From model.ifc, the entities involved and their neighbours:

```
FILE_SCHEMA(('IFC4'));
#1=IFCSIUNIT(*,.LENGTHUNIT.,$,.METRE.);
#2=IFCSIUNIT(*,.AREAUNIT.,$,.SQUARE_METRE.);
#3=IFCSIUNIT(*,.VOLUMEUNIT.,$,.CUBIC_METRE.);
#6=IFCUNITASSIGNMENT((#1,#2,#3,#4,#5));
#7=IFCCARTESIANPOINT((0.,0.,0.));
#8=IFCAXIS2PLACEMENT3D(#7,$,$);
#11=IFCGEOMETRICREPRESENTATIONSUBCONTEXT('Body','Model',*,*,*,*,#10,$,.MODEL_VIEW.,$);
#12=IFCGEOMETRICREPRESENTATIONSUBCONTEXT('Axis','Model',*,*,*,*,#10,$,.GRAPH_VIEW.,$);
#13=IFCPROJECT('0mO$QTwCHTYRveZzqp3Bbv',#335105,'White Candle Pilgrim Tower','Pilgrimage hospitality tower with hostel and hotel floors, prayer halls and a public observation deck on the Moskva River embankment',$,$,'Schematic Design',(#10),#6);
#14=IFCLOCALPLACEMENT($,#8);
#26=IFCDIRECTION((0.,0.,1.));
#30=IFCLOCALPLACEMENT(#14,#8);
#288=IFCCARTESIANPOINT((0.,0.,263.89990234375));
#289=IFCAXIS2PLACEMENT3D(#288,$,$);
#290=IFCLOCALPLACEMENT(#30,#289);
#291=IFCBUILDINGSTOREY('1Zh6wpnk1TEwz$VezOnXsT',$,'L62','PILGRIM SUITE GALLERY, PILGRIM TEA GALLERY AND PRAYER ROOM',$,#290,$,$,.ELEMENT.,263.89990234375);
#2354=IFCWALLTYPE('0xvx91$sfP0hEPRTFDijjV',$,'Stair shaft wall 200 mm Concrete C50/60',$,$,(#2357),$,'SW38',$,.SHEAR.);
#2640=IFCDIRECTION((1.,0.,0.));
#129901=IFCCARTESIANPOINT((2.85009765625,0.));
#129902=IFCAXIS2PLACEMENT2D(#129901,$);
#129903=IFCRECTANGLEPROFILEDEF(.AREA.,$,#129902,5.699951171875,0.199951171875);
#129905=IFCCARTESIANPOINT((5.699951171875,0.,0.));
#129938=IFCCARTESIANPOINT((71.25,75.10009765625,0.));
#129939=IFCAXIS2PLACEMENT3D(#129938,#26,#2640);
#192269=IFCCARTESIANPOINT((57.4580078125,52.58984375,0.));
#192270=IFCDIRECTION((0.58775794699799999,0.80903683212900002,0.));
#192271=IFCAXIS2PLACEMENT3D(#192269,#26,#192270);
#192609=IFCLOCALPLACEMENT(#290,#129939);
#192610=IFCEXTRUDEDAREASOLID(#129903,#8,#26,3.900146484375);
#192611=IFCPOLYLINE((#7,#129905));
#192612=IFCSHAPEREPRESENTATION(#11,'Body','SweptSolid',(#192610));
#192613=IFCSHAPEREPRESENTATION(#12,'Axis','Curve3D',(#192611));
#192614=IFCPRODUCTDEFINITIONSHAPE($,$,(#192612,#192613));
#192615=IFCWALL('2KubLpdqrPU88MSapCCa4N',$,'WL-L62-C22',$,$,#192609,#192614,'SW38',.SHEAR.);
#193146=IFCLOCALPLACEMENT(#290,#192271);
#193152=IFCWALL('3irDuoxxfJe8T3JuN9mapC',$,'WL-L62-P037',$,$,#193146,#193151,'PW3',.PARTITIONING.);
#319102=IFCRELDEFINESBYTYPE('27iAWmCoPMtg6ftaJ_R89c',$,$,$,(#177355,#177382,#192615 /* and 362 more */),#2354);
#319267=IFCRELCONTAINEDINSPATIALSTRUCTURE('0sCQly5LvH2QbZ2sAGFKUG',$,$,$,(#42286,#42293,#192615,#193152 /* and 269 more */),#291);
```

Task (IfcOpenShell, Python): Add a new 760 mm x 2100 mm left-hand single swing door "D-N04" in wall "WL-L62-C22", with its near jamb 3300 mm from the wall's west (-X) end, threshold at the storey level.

```python
import numpy as np
import ifcopenshell
import ifcopenshell.api.feature
import ifcopenshell.api.geometry
import ifcopenshell.api.root
import ifcopenshell.api.spatial
import ifcopenshell.geom
import ifcopenshell.util.element
import ifcopenshell.util.placement
import ifcopenshell.util.representation
import ifcopenshell.util.shape
import ifcopenshell.util.unit

model = ifcopenshell.open("model.ifc")
unit_scale = ifcopenshell.util.unit.calculate_unit_scale(model)
settings = ifcopenshell.geom.settings()


def volume(element):
    """Net volume in cubic metres, openings subtracted."""
    shape = ifcopenshell.geom.create_shape(settings, element)
    return ifcopenshell.util.shape.get_volume(shape.geometry)


wall = model.by_guid("2KubLpdqrPU88MSapCCa4N")
storey = ifcopenshell.util.element.get_container(wall, ifc_class="IfcBuildingStorey")
context = ifcopenshell.util.representation.get_context(model, "Model", "Body", "MODEL_VIEW")
before = volume(wall)

width, height, from_end, sill = 0.76, 2.1, 3.3, 0.0  # metres

# The wall runs along its own X axis, and the end named is its -X end.
wall_shape = ifcopenshell.geom.create_shape(settings, wall)
x, y, z = ifcopenshell.util.shape.get_vertices(wall_shape.geometry).T
start = x.min() + from_end
face, thickness = float(y.min()), float(y.max() - y.min())
wall_matrix = ifcopenshell.util.placement.get_local_placement(wall.ObjectPlacement)
level = ifcopenshell.util.placement.get_local_placement(storey.ObjectPlacement)[2, 3]


def in_wall(x, y):
    """Placement at x, y metres in the wall's axes, at sill height."""
    matrix = wall_matrix.copy()
    matrix[:, 3] = wall_matrix @ np.array([x / unit_scale, y / unit_scale, 0.0, 1.0])
    matrix[2, 3] = level + sill / unit_scale
    return matrix


# Opening: a box that overshoots both wall faces by 50 mm.
opening = ifcopenshell.api.root.create_entity(model, ifc_class="IfcOpeningElement", predefined_type="OPENING")
box = ifcopenshell.api.geometry.add_wall_representation(
    model, context=context, length=width, height=height, thickness=thickness + 0.1
)
ifcopenshell.api.geometry.assign_representation(model, product=opening, representation=box)
ifcopenshell.api.geometry.edit_object_placement(model, product=opening, matrix=in_wall(start, face - 0.05), is_si=False)
ifcopenshell.api.feature.add_feature(model, feature=opening, element=wall)

door = ifcopenshell.api.root.create_entity(model, ifc_class="IfcDoor", name="D-N04", predefined_type="DOOR")
door.OverallWidth, door.OverallHeight = width / unit_scale, height / unit_scale
door.OperationType = "SINGLE_SWING_LEFT"
body = ifcopenshell.api.geometry.add_door_representation(
    model,
    context=context,
    overall_width=door.OverallWidth,
    overall_height=door.OverallHeight,
    operation_type="SINGLE_SWING_LEFT",
    lining_properties={"LiningDepth": thickness / unit_scale, "ThresholdDepth": thickness / unit_scale},
)
ifcopenshell.api.geometry.assign_representation(model, product=door, representation=body)
ifcopenshell.api.spatial.assign_container(model, products=[door], relating_structure=storey)
ifcopenshell.api.feature.add_filling(model, opening=opening, element=door)

# The lining spans the wall, so the door starts at the wall face.
ifcopenshell.api.geometry.edit_object_placement(model, product=door, matrix=in_wall(start, face), is_si=False)

after = volume(wall)

print(f"wall volume {before:.3f} -> {after:.3f} m3")

model.write("model_rev.ifc")
```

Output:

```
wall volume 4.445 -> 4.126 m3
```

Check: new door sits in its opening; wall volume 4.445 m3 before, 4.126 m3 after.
